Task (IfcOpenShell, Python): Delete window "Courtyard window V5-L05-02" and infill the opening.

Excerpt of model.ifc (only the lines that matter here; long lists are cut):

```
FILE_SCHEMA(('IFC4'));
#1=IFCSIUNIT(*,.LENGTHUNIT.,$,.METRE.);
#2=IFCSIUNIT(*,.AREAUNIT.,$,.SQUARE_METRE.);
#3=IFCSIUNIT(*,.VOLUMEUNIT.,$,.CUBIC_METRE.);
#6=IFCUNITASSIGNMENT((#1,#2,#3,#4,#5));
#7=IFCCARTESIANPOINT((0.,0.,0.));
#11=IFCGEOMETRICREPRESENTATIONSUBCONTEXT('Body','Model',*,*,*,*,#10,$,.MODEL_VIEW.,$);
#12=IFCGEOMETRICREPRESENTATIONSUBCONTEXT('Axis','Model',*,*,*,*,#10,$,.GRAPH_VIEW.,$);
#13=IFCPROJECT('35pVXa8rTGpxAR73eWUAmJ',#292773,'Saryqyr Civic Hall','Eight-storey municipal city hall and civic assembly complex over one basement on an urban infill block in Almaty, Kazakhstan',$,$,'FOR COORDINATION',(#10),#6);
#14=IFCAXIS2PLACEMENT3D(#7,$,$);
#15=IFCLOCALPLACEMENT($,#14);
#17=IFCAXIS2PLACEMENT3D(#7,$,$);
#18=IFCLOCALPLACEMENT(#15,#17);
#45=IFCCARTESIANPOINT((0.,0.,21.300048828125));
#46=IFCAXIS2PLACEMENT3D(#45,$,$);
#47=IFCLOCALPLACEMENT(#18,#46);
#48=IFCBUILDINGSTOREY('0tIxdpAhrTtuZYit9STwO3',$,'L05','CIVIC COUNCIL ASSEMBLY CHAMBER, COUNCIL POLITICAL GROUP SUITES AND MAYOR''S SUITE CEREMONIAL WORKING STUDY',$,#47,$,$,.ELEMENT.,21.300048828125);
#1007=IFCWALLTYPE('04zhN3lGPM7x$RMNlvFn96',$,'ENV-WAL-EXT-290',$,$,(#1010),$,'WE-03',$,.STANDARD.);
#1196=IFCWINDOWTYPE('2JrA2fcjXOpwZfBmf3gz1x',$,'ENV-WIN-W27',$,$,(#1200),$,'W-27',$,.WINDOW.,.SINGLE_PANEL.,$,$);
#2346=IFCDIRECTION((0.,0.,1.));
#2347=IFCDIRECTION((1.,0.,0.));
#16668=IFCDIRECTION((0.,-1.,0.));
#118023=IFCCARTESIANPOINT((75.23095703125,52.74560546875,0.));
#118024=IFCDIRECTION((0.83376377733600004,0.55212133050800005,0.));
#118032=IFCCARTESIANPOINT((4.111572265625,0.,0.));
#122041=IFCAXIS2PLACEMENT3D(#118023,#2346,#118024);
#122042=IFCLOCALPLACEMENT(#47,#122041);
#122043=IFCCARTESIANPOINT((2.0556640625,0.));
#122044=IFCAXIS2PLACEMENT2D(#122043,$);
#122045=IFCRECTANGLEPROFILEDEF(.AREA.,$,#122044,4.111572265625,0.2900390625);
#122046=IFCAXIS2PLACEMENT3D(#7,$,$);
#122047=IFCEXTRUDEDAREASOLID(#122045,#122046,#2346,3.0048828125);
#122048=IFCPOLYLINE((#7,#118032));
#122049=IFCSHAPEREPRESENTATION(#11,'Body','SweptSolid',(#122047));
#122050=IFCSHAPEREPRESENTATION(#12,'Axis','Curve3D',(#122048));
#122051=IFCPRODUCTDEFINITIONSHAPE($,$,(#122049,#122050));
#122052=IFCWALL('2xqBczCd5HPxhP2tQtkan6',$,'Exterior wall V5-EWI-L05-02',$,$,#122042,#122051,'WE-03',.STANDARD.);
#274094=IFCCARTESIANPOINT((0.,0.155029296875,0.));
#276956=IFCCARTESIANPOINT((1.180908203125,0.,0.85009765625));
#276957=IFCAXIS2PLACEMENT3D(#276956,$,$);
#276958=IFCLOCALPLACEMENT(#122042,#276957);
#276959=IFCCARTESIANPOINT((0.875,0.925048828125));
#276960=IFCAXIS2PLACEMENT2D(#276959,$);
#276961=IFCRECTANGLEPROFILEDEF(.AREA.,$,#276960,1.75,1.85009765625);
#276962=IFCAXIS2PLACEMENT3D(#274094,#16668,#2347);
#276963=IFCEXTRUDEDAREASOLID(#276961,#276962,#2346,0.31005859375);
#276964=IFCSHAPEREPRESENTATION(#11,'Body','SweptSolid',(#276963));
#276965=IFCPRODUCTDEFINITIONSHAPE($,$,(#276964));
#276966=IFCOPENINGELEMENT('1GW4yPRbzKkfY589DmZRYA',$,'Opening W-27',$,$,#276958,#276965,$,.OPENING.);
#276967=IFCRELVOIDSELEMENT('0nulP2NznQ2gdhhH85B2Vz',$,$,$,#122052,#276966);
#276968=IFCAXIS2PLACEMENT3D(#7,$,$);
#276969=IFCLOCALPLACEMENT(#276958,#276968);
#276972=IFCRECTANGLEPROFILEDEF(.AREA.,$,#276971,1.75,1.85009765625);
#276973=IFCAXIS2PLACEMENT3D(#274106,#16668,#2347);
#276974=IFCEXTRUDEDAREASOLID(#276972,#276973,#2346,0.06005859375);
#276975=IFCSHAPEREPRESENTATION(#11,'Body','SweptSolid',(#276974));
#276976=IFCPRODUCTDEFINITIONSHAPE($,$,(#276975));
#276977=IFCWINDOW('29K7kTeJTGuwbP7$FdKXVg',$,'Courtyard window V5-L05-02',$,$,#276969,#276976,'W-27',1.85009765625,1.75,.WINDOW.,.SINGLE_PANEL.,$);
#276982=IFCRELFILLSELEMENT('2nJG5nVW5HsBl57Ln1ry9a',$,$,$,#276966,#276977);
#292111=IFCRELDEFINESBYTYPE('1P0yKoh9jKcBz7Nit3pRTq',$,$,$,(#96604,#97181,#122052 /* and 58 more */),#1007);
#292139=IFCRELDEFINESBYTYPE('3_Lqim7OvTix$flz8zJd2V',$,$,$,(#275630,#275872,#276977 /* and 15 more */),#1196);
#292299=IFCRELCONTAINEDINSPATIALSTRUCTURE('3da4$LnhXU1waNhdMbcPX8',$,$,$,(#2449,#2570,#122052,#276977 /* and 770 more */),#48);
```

```python
import ifcopenshell
import ifcopenshell.api.feature
import ifcopenshell.api.root
import ifcopenshell.geom
import ifcopenshell.util.shape

model = ifcopenshell.open("model.ifc")
settings = ifcopenshell.geom.settings()


def volume(element):
    """Net volume in cubic metres, openings subtracted."""
    shape = ifcopenshell.geom.create_shape(settings, element)
    return ifcopenshell.util.shape.get_volume(shape.geometry)


window = model.by_guid("29K7kTeJTGuwbP7$FdKXVg")
opening = window.FillsVoids[0].RelatingOpeningElement
wall = opening.VoidsElements[0].RelatingBuildingElement
before = volume(wall)

ifcopenshell.api.root.remove_product(model, product=window)
ifcopenshell.api.feature.remove_feature(model, feature=opening)

after = volume(wall)

print(f"wall volume {before:.3f} -> {after:.3f} m3")

model.write("model-out.ifc")
```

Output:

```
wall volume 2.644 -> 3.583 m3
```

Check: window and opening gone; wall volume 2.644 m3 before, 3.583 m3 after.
